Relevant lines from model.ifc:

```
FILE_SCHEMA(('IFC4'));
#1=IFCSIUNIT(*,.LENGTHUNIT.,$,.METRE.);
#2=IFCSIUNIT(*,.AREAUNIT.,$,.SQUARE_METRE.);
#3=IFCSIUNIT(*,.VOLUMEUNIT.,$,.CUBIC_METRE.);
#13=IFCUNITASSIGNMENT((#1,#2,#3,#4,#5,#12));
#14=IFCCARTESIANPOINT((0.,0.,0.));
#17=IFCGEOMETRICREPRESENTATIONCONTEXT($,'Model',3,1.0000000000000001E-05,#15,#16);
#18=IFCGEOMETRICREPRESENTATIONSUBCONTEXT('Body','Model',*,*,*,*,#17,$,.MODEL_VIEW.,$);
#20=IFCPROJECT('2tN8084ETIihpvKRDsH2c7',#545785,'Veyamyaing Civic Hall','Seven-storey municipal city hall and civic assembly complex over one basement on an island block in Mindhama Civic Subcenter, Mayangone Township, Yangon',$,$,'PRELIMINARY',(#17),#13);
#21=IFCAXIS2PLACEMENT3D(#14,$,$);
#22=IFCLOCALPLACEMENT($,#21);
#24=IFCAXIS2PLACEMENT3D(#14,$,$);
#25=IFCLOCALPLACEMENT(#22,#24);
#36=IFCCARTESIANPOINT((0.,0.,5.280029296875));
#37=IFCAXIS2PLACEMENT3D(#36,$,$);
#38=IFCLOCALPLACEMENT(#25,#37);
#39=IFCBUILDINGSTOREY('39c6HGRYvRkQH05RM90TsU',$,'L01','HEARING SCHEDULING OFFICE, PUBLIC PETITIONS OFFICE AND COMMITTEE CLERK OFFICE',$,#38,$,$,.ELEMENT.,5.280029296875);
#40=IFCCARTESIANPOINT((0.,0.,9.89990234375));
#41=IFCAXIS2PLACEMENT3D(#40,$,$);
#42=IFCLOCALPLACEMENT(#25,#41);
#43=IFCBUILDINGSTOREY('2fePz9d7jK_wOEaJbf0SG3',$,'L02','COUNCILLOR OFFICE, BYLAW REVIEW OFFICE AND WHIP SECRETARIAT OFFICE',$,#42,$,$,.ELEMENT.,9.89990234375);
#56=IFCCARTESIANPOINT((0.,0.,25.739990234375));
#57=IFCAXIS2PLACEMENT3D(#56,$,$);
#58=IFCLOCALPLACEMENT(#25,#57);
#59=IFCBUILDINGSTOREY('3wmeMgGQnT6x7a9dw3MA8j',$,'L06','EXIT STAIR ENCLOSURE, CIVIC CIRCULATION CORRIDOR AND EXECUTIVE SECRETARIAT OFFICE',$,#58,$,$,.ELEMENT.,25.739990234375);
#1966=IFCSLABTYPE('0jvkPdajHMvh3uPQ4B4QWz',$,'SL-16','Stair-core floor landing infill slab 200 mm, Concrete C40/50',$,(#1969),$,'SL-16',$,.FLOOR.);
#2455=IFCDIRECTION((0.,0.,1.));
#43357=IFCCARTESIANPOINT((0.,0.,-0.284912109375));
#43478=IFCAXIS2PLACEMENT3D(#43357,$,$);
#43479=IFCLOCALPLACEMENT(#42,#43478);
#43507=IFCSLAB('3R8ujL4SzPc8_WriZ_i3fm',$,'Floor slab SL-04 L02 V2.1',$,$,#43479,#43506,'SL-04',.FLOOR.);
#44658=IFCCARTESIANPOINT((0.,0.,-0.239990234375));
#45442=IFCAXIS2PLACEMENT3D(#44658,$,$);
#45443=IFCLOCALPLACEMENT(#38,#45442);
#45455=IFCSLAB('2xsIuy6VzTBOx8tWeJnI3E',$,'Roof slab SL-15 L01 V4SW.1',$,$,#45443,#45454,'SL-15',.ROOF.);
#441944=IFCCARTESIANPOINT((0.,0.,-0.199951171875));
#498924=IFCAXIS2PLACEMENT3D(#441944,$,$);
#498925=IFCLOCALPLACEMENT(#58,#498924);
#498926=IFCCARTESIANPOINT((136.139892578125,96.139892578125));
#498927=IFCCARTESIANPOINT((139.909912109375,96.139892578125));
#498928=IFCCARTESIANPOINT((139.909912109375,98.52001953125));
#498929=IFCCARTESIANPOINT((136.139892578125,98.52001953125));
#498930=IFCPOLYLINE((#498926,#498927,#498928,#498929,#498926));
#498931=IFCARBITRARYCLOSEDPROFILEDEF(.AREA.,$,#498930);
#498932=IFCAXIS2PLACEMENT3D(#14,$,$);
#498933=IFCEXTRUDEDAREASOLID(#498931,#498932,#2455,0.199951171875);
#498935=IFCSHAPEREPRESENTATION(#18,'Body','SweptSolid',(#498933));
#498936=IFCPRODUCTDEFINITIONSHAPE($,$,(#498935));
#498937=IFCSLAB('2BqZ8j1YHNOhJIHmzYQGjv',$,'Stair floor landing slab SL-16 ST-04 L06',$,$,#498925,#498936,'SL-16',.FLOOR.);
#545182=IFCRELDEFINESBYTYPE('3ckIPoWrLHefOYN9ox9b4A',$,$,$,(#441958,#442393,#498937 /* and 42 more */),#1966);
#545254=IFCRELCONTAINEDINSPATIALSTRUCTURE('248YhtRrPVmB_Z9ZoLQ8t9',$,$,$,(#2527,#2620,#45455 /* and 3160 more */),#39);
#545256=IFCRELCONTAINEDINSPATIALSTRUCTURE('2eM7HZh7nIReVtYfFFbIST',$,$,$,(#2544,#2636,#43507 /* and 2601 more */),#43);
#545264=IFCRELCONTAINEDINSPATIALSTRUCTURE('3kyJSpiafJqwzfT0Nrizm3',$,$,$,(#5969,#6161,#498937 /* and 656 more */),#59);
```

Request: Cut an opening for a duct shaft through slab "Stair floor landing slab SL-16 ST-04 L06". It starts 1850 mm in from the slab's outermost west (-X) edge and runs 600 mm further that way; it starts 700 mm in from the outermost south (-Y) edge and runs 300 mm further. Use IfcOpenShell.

```python
import numpy as np
import ifcopenshell
import ifcopenshell.api.feature
import ifcopenshell.api.geometry
import ifcopenshell.api.root
import ifcopenshell.geom
import ifcopenshell.util.placement
import ifcopenshell.util.representation
import ifcopenshell.util.shape
import ifcopenshell.util.unit

model = ifcopenshell.open("model.ifc")
unit_scale = ifcopenshell.util.unit.calculate_unit_scale(model)
settings = ifcopenshell.geom.settings()


def volume(element):
    """Net volume in cubic metres, openings subtracted."""
    shape = ifcopenshell.geom.create_shape(settings, element)
    return ifcopenshell.util.shape.get_volume(shape.geometry)


slab = model.by_id(498937)
before = volume(slab)

# Extent in the slab's own axes, in metres. The edges named are its -X and -Y sides.
slab_shape = ifcopenshell.geom.create_shape(settings, slab)
vertices = ifcopenshell.util.shape.get_vertices(slab_shape.geometry)
x_min, y_min, bottom = vertices.min(axis=0)
top = vertices[:, 2].max()

opening = ifcopenshell.api.root.create_entity(model, ifc_class="IfcOpeningElement", name="Duct shaft opening", predefined_type="OPENING")
context = ifcopenshell.util.representation.get_context(model, "Model", "Body", "MODEL_VIEW")
width, depth = 0.6, 0.3
outline = [(0.0, 0.0), (width, 0.0), (width, depth), (0.0, depth), (0.0, 0.0)]
# Overshoot both faces by 50 mm so the cut is clean.
shape = ifcopenshell.api.geometry.add_slab_representation(
    model, context=context, depth=top - bottom + 0.1, polyline=outline
)
ifcopenshell.api.geometry.assign_representation(model, product=opening, representation=shape)

matrix = ifcopenshell.util.placement.get_local_placement(slab.ObjectPlacement)
matrix[:, 3] = matrix @ np.append(np.array([x_min + 1.85, y_min + 0.7, bottom - 0.05]) / unit_scale, 1.0)
ifcopenshell.api.geometry.edit_object_placement(model, product=opening, matrix=matrix, is_si=False)
ifcopenshell.api.feature.add_feature(model, feature=opening, element=slab)

after = volume(slab)

print(f"slab volume {before:.3f} -> {after:.3f} m3")

model.write("model-out.ifc")
```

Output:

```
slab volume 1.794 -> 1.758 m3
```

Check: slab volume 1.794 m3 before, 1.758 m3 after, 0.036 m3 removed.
